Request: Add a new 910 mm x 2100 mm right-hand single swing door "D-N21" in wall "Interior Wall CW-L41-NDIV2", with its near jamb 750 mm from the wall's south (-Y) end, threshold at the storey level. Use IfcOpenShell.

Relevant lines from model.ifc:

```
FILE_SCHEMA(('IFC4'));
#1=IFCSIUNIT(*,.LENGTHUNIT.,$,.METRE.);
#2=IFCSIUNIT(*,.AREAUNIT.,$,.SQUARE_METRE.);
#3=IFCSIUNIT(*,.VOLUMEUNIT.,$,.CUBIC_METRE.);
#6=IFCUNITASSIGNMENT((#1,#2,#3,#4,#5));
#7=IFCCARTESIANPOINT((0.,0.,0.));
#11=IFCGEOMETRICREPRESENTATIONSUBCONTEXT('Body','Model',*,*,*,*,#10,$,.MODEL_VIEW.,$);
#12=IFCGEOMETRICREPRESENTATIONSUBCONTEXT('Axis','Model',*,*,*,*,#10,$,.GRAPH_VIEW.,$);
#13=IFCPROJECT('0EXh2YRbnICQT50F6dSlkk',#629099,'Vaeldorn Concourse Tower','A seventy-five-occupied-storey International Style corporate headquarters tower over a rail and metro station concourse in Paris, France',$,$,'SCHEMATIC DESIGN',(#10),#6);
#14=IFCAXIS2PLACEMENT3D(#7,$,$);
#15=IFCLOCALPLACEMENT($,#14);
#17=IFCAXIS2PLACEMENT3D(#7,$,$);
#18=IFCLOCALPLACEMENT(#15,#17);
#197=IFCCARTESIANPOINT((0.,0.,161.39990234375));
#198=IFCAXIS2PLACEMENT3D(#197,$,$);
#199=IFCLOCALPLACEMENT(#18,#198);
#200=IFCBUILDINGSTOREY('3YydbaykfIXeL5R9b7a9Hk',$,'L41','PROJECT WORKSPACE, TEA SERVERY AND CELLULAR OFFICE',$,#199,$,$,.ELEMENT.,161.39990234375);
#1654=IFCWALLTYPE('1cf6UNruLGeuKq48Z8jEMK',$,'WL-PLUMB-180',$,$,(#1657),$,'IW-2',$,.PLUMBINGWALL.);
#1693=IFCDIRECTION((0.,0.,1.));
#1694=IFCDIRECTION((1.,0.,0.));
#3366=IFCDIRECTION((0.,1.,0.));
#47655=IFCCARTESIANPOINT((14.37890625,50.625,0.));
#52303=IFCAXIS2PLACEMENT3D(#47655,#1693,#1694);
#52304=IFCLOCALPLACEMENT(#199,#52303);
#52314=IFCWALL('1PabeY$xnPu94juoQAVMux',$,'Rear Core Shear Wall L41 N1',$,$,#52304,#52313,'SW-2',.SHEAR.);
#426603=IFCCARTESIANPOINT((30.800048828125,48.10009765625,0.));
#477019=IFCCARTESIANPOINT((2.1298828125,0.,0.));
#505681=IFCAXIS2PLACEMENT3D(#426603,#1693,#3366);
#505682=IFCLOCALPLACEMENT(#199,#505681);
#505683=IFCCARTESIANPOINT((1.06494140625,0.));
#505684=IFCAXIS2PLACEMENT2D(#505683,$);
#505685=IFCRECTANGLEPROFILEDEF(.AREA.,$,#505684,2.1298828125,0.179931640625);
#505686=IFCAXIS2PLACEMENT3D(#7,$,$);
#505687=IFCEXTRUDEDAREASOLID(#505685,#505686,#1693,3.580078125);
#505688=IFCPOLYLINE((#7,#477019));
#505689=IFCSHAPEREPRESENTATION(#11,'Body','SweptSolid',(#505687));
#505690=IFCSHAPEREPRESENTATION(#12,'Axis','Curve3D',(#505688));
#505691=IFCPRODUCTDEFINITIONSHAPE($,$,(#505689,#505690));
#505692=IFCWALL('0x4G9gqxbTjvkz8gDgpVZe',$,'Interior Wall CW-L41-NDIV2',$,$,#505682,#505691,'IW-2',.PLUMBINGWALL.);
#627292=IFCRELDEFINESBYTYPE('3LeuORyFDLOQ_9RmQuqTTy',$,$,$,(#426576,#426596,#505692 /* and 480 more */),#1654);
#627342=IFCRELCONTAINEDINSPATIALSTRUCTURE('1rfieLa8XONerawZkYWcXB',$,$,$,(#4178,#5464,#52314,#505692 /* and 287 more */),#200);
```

```python
import numpy as np
import ifcopenshell
import ifcopenshell.api.feature
import ifcopenshell.api.geometry
import ifcopenshell.api.root
import ifcopenshell.api.spatial
import ifcopenshell.geom
import ifcopenshell.util.element
import ifcopenshell.util.placement
import ifcopenshell.util.representation
import ifcopenshell.util.shape
import ifcopenshell.util.unit

model = ifcopenshell.open("model.ifc")
unit_scale = ifcopenshell.util.unit.calculate_unit_scale(model)
settings = ifcopenshell.geom.settings()


def volume(element):
    """Net volume in cubic metres, openings subtracted."""
    shape = ifcopenshell.geom.create_shape(settings, element)
    return ifcopenshell.util.shape.get_volume(shape.geometry)


wall = model.by_guid("0x4G9gqxbTjvkz8gDgpVZe")
storey = ifcopenshell.util.element.get_container(wall, ifc_class="IfcBuildingStorey")
context = ifcopenshell.util.representation.get_context(model, "Model", "Body", "MODEL_VIEW")
before = volume(wall)

width, height, from_end, sill = 0.91, 2.1, 0.75, 0.0  # metres

# The wall runs along its own X axis, and the end named is its -X end.
wall_shape = ifcopenshell.geom.create_shape(settings, wall)
x, y, z = ifcopenshell.util.shape.get_vertices(wall_shape.geometry).T
start = x.min() + from_end
face, thickness = float(y.min()), float(y.max() - y.min())
wall_matrix = ifcopenshell.util.placement.get_local_placement(wall.ObjectPlacement)
level = ifcopenshell.util.placement.get_local_placement(storey.ObjectPlacement)[2, 3]


def in_wall(x, y):
    """Placement at x, y metres in the wall's axes, at sill height."""
    matrix = wall_matrix.copy()
    matrix[:, 3] = wall_matrix @ np.array([x / unit_scale, y / unit_scale, 0.0, 1.0])
    matrix[2, 3] = level + sill / unit_scale
    return matrix


# Opening: a box that overshoots both wall faces by 50 mm.
opening = ifcopenshell.api.root.create_entity(model, ifc_class="IfcOpeningElement", predefined_type="OPENING")
box = ifcopenshell.api.geometry.add_wall_representation(
    model, context=context, length=width, height=height, thickness=thickness + 0.1
)
ifcopenshell.api.geometry.assign_representation(model, product=opening, representation=box)
ifcopenshell.api.geometry.edit_object_placement(model, product=opening, matrix=in_wall(start, face - 0.05), is_si=False)
ifcopenshell.api.feature.add_feature(model, feature=opening, element=wall)

door = ifcopenshell.api.root.create_entity(model, ifc_class="IfcDoor", name="D-N21", predefined_type="DOOR")
door.OverallWidth, door.OverallHeight = width / unit_scale, height / unit_scale
door.OperationType = "SINGLE_SWING_RIGHT"
body = ifcopenshell.api.geometry.add_door_representation(
    model,
    context=context,
    overall_width=door.OverallWidth,
    overall_height=door.OverallHeight,
    operation_type="SINGLE_SWING_RIGHT",
    lining_properties={"LiningDepth": thickness / unit_scale, "ThresholdDepth": thickness / unit_scale},
)
ifcopenshell.api.geometry.assign_representation(model, product=door, representation=body)
ifcopenshell.api.spatial.assign_container(model, products=[door], relating_structure=storey)
ifcopenshell.api.feature.add_filling(model, opening=opening, element=door)

# The lining spans the wall, so the door starts at the wall face.
ifcopenshell.api.geometry.edit_object_placement(model, product=door, matrix=in_wall(start, face), is_si=False)

after = volume(wall)

print(f"wall volume {before:.3f} -> {after:.3f} m3")

model.write("model_updated.ifc")
```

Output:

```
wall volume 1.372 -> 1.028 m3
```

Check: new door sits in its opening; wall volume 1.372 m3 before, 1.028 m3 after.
